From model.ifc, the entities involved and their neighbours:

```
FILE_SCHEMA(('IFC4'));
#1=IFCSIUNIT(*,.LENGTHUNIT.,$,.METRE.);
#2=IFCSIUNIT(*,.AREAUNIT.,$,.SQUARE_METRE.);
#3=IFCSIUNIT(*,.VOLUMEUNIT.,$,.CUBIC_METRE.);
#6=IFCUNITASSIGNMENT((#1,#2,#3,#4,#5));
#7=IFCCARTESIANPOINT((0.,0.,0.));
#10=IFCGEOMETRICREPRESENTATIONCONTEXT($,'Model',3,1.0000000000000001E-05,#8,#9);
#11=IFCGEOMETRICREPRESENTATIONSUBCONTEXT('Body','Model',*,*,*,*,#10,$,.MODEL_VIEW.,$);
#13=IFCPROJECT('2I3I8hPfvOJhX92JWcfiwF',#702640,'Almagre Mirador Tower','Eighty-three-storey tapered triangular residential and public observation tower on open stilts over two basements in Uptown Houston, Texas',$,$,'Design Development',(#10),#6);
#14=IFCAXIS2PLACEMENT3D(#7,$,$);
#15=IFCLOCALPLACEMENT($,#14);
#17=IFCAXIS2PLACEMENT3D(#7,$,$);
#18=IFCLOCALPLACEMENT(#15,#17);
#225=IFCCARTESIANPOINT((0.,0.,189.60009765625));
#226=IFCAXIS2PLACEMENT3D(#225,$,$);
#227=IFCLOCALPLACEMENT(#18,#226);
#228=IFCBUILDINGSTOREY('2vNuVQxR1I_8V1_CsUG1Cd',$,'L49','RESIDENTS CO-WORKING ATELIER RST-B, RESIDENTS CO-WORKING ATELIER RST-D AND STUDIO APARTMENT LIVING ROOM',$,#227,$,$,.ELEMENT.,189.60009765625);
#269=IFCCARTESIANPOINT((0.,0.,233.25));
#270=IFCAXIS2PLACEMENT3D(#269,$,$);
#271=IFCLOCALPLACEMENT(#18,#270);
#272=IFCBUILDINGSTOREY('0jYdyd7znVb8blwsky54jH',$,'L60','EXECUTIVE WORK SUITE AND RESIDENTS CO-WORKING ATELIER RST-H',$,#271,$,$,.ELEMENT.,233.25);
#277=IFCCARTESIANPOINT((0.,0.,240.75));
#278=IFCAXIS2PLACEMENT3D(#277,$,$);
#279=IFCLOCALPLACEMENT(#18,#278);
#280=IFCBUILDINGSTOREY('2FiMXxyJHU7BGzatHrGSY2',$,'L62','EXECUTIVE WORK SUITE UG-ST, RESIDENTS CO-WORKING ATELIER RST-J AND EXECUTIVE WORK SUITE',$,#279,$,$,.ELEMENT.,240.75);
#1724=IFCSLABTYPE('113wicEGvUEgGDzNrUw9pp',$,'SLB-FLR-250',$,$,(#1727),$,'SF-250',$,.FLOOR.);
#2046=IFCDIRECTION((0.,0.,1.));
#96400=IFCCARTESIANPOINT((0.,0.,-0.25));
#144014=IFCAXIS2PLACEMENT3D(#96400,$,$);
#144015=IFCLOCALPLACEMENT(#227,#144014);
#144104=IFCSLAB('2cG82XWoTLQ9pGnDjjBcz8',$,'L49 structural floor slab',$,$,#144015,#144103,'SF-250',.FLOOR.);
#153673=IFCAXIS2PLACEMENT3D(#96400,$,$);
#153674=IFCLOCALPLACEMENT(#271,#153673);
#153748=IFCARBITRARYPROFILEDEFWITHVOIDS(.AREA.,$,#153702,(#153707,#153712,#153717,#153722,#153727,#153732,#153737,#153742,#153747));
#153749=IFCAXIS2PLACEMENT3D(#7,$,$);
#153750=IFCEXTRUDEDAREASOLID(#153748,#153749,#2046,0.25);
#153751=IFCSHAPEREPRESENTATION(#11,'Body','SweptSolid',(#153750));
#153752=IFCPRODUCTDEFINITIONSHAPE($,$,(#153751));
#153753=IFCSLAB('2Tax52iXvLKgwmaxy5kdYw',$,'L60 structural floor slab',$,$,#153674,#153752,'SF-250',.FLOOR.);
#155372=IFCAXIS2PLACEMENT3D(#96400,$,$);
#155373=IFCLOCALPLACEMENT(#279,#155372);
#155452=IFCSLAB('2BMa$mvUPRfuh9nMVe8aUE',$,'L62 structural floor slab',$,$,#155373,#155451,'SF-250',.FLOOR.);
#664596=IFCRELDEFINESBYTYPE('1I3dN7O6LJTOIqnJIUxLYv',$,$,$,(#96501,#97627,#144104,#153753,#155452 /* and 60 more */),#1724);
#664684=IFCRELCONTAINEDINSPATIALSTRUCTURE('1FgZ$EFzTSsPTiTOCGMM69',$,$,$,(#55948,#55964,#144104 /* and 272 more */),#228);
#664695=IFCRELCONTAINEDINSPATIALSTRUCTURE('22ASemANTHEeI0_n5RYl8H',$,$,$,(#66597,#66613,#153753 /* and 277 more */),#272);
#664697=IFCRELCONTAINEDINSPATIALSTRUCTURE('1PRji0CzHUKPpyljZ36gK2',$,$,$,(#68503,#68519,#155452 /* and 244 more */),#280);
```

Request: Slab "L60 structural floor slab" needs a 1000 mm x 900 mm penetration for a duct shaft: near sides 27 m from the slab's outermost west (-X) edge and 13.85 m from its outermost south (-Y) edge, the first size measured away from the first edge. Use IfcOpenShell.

```python
import numpy as np
import ifcopenshell
import ifcopenshell.api.feature
import ifcopenshell.api.geometry
import ifcopenshell.api.root
import ifcopenshell.geom
import ifcopenshell.util.placement
import ifcopenshell.util.representation
import ifcopenshell.util.shape
import ifcopenshell.util.unit

model = ifcopenshell.open("model.ifc")
unit_scale = ifcopenshell.util.unit.calculate_unit_scale(model)
settings = ifcopenshell.geom.settings()


def volume(element):
    """Net volume in cubic metres, openings subtracted."""
    shape = ifcopenshell.geom.create_shape(settings, element)
    return ifcopenshell.util.shape.get_volume(shape.geometry)


slab = model.by_guid("2Tax52iXvLKgwmaxy5kdYw")
before = volume(slab)

# Extent in the slab's own axes, in metres. The edges named are its -X and -Y sides.
slab_shape = ifcopenshell.geom.create_shape(settings, slab)
vertices = ifcopenshell.util.shape.get_vertices(slab_shape.geometry)
x_min, y_min, bottom = vertices.min(axis=0)
top = vertices[:, 2].max()

opening = ifcopenshell.api.root.create_entity(model, ifc_class="IfcOpeningElement", name="Duct shaft opening", predefined_type="OPENING")
context = ifcopenshell.util.representation.get_context(model, "Model", "Body", "MODEL_VIEW")
width, depth = 1, 0.9
outline = [(0.0, 0.0), (width, 0.0), (width, depth), (0.0, depth), (0.0, 0.0)]
# Overshoot both faces by 50 mm so the cut is clean.
shape = ifcopenshell.api.geometry.add_slab_representation(
    model, context=context, depth=top - bottom + 0.1, polyline=outline
)
ifcopenshell.api.geometry.assign_representation(model, product=opening, representation=shape)

matrix = ifcopenshell.util.placement.get_local_placement(slab.ObjectPlacement)
matrix[:, 3] = matrix @ np.append(np.array([x_min + 27, y_min + 13.85, bottom - 0.05]) / unit_scale, 1.0)
ifcopenshell.api.geometry.edit_object_placement(model, product=opening, matrix=matrix, is_si=False)
ifcopenshell.api.feature.add_feature(model, feature=opening, element=slab)

after = volume(slab)

print(f"slab volume {before:.3f} -> {after:.3f} m3")

model.write("model_rev.ifc")
```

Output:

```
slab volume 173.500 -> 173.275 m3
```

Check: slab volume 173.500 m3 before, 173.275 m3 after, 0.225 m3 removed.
